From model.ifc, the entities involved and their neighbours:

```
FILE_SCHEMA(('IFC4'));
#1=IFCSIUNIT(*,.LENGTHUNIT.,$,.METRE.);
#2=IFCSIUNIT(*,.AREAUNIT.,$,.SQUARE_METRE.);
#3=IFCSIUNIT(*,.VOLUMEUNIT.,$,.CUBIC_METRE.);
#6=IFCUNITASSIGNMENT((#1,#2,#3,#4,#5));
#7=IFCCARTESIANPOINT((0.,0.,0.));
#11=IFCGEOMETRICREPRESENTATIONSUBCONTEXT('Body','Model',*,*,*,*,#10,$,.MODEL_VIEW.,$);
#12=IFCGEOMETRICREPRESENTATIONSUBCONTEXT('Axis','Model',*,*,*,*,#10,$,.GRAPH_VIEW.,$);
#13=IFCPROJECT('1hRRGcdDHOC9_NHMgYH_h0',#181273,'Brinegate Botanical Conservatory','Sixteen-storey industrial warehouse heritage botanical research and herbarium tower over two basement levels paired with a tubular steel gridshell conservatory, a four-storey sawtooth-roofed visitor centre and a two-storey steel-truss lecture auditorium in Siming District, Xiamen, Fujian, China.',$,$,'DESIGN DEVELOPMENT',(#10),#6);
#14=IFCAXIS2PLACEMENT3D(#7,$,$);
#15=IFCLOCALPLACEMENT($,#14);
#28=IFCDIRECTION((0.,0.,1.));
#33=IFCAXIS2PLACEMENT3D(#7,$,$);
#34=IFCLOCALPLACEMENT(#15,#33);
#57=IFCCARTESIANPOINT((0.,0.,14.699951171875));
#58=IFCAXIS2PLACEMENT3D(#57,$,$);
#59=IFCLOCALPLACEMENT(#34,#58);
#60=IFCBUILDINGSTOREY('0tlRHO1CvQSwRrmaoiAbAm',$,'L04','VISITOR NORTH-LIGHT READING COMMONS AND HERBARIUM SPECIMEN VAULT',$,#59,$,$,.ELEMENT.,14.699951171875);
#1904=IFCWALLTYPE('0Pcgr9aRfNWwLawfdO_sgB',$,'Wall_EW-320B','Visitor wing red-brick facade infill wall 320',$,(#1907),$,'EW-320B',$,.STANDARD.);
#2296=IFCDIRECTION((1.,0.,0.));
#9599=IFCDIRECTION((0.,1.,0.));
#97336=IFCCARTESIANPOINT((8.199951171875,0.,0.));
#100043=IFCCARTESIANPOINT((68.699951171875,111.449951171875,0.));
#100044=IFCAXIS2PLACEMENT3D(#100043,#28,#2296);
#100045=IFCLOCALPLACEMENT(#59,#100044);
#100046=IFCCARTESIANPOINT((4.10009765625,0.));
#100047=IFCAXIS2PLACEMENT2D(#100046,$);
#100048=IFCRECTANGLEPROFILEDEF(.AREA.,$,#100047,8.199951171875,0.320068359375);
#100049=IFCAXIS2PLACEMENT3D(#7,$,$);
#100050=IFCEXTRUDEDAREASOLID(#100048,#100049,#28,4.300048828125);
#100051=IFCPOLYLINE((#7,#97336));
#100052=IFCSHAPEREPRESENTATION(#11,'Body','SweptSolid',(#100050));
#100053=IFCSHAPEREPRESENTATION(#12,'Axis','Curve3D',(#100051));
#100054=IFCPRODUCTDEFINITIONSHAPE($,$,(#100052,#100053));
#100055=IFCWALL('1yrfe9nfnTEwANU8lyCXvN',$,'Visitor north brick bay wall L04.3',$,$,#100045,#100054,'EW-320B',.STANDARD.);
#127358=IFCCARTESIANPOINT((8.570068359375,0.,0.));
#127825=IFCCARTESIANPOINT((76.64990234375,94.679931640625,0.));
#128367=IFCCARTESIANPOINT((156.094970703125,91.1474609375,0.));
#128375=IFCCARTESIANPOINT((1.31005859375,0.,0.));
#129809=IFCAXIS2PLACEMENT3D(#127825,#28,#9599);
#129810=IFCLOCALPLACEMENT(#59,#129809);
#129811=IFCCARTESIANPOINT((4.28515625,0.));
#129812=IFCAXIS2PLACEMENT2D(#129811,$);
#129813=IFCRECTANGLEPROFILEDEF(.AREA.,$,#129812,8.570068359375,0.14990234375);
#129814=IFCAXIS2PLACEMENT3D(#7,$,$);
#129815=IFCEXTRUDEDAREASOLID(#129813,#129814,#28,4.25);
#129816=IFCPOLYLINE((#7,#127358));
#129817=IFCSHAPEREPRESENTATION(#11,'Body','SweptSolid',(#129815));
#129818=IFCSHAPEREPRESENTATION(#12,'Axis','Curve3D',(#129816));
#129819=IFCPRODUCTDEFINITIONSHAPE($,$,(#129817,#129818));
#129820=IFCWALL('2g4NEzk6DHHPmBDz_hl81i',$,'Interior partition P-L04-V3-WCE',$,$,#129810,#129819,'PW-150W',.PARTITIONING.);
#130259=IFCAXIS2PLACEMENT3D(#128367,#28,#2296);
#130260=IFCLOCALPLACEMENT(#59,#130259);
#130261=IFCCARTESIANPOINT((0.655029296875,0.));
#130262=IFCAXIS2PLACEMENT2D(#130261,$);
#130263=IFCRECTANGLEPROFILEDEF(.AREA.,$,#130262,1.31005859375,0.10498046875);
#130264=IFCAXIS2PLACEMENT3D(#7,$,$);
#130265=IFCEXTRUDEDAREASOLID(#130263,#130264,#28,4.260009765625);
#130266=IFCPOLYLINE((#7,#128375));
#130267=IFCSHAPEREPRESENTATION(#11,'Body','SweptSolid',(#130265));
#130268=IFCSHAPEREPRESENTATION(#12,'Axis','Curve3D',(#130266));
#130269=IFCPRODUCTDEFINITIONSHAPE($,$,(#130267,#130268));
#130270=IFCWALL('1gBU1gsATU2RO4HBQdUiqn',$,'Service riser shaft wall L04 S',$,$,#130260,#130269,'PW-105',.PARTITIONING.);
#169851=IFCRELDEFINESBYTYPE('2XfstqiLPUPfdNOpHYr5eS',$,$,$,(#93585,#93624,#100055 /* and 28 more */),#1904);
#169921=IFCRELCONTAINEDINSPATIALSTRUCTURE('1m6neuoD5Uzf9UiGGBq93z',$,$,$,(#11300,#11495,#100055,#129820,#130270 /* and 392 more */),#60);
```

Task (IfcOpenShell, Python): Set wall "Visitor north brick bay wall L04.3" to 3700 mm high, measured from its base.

```python
import ifcopenshell
import ifcopenshell.geom
import ifcopenshell.util.representation
import ifcopenshell.util.shape

model = ifcopenshell.open("model.ifc")
settings = ifcopenshell.geom.settings()


def volume(element):
    """Net volume in cubic metres, openings subtracted."""
    shape = ifcopenshell.geom.create_shape(settings, element)
    return ifcopenshell.util.shape.get_volume(shape.geometry)


wall = model.by_guid("1yrfe9nfnTEwANU8lyCXvN")
before = volume(wall)

body = ifcopenshell.util.representation.get_representation(wall, "Model", "Body")
solid = body.Items[0]
old_height = solid.Depth
solid.Depth = 3.7
after = volume(wall)

print(f"height {old_height:g} -> {solid.Depth:g}, volume {before:.3f} -> {after:.3f} m3")

model.write("model_rev.ifc")
```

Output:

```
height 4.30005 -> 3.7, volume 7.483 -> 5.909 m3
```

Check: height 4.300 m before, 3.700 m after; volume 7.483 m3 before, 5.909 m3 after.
